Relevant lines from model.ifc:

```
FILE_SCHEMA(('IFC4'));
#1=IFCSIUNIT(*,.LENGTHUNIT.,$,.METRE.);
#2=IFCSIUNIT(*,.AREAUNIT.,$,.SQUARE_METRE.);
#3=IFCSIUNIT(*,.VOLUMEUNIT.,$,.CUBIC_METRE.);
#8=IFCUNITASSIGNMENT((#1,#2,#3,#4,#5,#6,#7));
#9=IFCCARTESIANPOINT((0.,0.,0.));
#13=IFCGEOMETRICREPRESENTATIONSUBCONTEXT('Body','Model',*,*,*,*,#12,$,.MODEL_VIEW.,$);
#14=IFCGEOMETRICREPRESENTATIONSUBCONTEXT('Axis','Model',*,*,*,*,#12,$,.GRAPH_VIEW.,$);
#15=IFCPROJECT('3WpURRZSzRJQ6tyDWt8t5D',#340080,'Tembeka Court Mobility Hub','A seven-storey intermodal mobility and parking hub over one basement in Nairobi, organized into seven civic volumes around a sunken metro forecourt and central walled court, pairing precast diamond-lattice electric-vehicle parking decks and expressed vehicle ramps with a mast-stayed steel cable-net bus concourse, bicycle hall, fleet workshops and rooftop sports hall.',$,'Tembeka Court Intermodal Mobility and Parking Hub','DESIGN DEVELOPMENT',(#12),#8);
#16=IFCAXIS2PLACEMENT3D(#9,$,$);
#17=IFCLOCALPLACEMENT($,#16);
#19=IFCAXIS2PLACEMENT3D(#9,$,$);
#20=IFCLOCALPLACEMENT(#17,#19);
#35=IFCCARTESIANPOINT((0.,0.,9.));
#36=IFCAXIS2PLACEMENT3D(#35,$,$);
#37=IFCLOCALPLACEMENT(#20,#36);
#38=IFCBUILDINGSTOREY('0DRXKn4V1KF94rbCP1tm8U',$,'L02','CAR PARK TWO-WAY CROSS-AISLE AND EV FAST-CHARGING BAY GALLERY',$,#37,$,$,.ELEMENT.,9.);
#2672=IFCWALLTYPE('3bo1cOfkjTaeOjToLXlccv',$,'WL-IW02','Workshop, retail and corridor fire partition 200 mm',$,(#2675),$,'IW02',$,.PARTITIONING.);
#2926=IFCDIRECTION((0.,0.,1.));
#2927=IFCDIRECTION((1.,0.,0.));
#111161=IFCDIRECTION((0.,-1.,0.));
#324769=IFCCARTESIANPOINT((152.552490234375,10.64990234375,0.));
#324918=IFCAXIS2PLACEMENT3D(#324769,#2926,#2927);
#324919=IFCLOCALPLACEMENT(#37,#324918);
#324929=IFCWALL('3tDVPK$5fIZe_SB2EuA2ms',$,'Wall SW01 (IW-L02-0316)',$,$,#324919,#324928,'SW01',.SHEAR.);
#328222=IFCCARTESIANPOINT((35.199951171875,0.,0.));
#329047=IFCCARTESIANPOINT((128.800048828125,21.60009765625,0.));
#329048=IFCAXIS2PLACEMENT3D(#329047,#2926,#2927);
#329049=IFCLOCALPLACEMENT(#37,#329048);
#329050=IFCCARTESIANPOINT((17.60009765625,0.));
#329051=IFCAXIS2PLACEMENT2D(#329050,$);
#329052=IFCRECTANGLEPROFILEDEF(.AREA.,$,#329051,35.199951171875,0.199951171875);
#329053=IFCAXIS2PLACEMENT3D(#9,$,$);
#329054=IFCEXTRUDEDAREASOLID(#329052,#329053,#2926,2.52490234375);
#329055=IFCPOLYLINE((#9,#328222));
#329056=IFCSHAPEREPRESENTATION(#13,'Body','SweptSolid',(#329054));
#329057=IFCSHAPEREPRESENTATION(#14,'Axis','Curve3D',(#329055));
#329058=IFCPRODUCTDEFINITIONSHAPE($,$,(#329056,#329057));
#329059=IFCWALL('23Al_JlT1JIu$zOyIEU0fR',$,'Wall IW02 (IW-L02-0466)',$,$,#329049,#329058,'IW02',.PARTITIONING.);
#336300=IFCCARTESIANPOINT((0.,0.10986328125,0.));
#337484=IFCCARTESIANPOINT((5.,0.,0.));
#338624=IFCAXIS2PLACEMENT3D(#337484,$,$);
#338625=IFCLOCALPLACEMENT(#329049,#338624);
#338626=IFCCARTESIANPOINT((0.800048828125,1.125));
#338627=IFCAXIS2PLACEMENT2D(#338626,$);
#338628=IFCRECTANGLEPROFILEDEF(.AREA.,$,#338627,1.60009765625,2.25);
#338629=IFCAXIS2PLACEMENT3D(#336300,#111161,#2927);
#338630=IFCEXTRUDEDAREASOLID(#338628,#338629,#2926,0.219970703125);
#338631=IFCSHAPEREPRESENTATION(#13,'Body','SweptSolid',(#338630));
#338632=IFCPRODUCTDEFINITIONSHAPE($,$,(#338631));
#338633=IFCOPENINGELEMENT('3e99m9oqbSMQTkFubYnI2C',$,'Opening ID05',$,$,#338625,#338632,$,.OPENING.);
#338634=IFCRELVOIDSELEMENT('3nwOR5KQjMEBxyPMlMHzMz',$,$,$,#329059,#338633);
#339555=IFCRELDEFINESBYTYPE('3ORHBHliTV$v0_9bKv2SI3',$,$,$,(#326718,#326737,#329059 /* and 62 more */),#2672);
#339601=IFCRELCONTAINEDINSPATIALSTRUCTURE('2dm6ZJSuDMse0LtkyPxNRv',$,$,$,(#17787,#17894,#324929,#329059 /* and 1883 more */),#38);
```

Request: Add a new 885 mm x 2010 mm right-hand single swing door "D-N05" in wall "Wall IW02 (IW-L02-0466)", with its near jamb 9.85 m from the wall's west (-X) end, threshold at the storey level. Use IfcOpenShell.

```python
import numpy as np
import ifcopenshell
import ifcopenshell.api.feature
import ifcopenshell.api.geometry
import ifcopenshell.api.root
import ifcopenshell.api.spatial
import ifcopenshell.geom
import ifcopenshell.util.element
import ifcopenshell.util.placement
import ifcopenshell.util.representation
import ifcopenshell.util.shape
import ifcopenshell.util.unit

model = ifcopenshell.open("model.ifc")
unit_scale = ifcopenshell.util.unit.calculate_unit_scale(model)
settings = ifcopenshell.geom.settings()


def volume(element):
    """Net volume in cubic metres, openings subtracted."""
    shape = ifcopenshell.geom.create_shape(settings, element)
    return ifcopenshell.util.shape.get_volume(shape.geometry)


wall = model.by_guid("23Al_JlT1JIu$zOyIEU0fR")
storey = ifcopenshell.util.element.get_container(wall, ifc_class="IfcBuildingStorey")
context = ifcopenshell.util.representation.get_context(model, "Model", "Body", "MODEL_VIEW")
before = volume(wall)

width, height, from_end, sill = 0.885, 2.01, 9.85, 0.0  # metres

# The wall runs along its own X axis, and the end named is its -X end.
wall_shape = ifcopenshell.geom.create_shape(settings, wall)
x, y, z = ifcopenshell.util.shape.get_vertices(wall_shape.geometry).T
start = x.min() + from_end
face, thickness = float(y.min()), float(y.max() - y.min())
wall_matrix = ifcopenshell.util.placement.get_local_placement(wall.ObjectPlacement)
level = ifcopenshell.util.placement.get_local_placement(storey.ObjectPlacement)[2, 3]


def in_wall(x, y):
    """Placement at x, y metres in the wall's axes, at sill height."""
    matrix = wall_matrix.copy()
    matrix[:, 3] = wall_matrix @ np.array([x / unit_scale, y / unit_scale, 0.0, 1.0])
    matrix[2, 3] = level + sill / unit_scale
    return matrix


# Opening: a box that overshoots both wall faces by 50 mm.
opening = ifcopenshell.api.root.create_entity(model, ifc_class="IfcOpeningElement", predefined_type="OPENING")
box = ifcopenshell.api.geometry.add_wall_representation(
    model, context=context, length=width, height=height, thickness=thickness + 0.1
)
ifcopenshell.api.geometry.assign_representation(model, product=opening, representation=box)
ifcopenshell.api.geometry.edit_object_placement(model, product=opening, matrix=in_wall(start, face - 0.05), is_si=False)
ifcopenshell.api.feature.add_feature(model, feature=opening, element=wall)

door = ifcopenshell.api.root.create_entity(model, ifc_class="IfcDoor", name="D-N05", predefined_type="DOOR")
door.OverallWidth, door.OverallHeight = width / unit_scale, height / unit_scale
door.OperationType = "SINGLE_SWING_RIGHT"
body = ifcopenshell.api.geometry.add_door_representation(
    model,
    context=context,
    overall_width=door.OverallWidth,
    overall_height=door.OverallHeight,
    operation_type="SINGLE_SWING_RIGHT",
    lining_properties={"LiningDepth": thickness / unit_scale, "ThresholdDepth": thickness / unit_scale},
)
ifcopenshell.api.geometry.assign_representation(model, product=door, representation=body)
ifcopenshell.api.spatial.assign_container(model, products=[door], relating_structure=storey)
ifcopenshell.api.feature.add_filling(model, opening=opening, element=door)

# The lining spans the wall, so the door starts at the wall face.
ifcopenshell.api.geometry.edit_object_placement(model, product=door, matrix=in_wall(start, face), is_si=False)

after = volume(wall)

print(f"wall volume {before:.3f} -> {after:.3f} m3")

model.write("model_v2.ifc")
```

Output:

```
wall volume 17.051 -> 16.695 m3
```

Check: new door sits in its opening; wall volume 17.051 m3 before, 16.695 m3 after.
